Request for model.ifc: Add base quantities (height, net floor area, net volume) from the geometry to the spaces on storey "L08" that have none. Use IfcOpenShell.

First a look at what the model holds.

```python
import ifcopenshell
import ifcopenshell.util.element
import ifcopenshell.util.unit

model = ifcopenshell.open("model.ifc")
print(model.schema)
for unit_type in ("LENGTHUNIT", "AREAUNIT", "VOLUMEUNIT"):
    print(unit_type, ifcopenshell.util.unit.calculate_unit_scale(model, unit_type))
storey = next(s for s in model.by_type("IfcBuildingStorey") if s.Name == "L08")
spaces = [e for e in ifcopenshell.util.element.get_decomposition(storey) if e.is_a("IfcSpace")]
for e in sorted(spaces, key=lambda e: e.id()):
    print(e.id(), e.is_a(), e.Name, list(ifcopenshell.util.element.get_psets(e, qtos_only=True)), sep=" | ")
```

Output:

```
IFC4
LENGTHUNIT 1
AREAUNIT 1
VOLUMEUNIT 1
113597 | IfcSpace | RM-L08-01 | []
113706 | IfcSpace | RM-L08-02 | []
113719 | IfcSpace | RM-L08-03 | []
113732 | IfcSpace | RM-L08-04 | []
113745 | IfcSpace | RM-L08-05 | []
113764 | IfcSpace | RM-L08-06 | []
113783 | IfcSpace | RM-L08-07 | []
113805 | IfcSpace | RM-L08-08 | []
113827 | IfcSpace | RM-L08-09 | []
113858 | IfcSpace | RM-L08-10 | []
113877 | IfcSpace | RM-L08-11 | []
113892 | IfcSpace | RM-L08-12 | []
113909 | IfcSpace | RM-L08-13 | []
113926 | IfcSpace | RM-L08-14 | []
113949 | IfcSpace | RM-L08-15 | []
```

```python
import ifcopenshell
import ifcopenshell.api.pset
import ifcopenshell.geom
import ifcopenshell.util.element
import ifcopenshell.util.shape
import ifcopenshell.util.unit

model = ifcopenshell.open("model.ifc")
unit_scale = ifcopenshell.util.unit.calculate_unit_scale(model)
area_scale = ifcopenshell.util.unit.calculate_unit_scale(model, "AREAUNIT")
volume_scale = ifcopenshell.util.unit.calculate_unit_scale(model, "VOLUMEUNIT")
settings = ifcopenshell.geom.settings()

storey = next(s for s in model.by_type("IfcBuildingStorey") if s.Name == "L08")
spaces = [e for e in ifcopenshell.util.element.get_decomposition(storey) if e.is_a("IfcSpace")]

for e in sorted(spaces, key=lambda e: e.id()):
    if ifcopenshell.util.element.get_psets(e, qtos_only=True, should_inherit=False):
        continue
    # Geometry comes back in metres, in the element's own axes.
    shape = ifcopenshell.geom.create_shape(settings, e)
    values = {
        "Height": ifcopenshell.util.shape.get_z(shape.geometry) / unit_scale,
        "NetFloorArea": ifcopenshell.util.shape.get_footprint_area(shape.geometry) / area_scale,
        "NetVolume": ifcopenshell.util.shape.get_volume(shape.geometry) / volume_scale,
    }
    qto = ifcopenshell.api.pset.add_qto(model, product=e, name="Qto_SpaceBaseQuantities")
    ifcopenshell.api.pset.edit_qto(model, qto=qto, properties=values)
    print(e.id(), {k: round(v, 3) for k, v in values.items()})

model.write("model_rev.ifc")
```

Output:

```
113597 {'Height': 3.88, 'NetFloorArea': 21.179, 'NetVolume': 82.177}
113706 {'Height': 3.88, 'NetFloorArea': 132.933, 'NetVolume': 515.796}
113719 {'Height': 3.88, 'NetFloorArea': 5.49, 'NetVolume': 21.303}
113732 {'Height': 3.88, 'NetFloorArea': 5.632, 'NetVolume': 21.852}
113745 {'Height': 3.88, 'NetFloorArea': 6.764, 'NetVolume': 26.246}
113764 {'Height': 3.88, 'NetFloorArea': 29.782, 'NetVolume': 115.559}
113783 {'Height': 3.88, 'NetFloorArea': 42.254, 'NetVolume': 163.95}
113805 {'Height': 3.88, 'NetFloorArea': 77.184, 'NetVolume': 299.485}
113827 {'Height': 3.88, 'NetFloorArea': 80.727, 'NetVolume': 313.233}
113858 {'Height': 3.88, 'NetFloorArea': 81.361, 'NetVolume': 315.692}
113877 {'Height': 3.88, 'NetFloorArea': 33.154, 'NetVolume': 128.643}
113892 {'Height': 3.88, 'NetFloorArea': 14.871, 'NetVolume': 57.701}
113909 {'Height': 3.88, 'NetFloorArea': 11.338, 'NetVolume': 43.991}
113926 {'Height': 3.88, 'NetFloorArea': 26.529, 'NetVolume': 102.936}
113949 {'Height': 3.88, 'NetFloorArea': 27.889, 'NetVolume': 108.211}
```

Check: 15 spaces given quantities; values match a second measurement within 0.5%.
